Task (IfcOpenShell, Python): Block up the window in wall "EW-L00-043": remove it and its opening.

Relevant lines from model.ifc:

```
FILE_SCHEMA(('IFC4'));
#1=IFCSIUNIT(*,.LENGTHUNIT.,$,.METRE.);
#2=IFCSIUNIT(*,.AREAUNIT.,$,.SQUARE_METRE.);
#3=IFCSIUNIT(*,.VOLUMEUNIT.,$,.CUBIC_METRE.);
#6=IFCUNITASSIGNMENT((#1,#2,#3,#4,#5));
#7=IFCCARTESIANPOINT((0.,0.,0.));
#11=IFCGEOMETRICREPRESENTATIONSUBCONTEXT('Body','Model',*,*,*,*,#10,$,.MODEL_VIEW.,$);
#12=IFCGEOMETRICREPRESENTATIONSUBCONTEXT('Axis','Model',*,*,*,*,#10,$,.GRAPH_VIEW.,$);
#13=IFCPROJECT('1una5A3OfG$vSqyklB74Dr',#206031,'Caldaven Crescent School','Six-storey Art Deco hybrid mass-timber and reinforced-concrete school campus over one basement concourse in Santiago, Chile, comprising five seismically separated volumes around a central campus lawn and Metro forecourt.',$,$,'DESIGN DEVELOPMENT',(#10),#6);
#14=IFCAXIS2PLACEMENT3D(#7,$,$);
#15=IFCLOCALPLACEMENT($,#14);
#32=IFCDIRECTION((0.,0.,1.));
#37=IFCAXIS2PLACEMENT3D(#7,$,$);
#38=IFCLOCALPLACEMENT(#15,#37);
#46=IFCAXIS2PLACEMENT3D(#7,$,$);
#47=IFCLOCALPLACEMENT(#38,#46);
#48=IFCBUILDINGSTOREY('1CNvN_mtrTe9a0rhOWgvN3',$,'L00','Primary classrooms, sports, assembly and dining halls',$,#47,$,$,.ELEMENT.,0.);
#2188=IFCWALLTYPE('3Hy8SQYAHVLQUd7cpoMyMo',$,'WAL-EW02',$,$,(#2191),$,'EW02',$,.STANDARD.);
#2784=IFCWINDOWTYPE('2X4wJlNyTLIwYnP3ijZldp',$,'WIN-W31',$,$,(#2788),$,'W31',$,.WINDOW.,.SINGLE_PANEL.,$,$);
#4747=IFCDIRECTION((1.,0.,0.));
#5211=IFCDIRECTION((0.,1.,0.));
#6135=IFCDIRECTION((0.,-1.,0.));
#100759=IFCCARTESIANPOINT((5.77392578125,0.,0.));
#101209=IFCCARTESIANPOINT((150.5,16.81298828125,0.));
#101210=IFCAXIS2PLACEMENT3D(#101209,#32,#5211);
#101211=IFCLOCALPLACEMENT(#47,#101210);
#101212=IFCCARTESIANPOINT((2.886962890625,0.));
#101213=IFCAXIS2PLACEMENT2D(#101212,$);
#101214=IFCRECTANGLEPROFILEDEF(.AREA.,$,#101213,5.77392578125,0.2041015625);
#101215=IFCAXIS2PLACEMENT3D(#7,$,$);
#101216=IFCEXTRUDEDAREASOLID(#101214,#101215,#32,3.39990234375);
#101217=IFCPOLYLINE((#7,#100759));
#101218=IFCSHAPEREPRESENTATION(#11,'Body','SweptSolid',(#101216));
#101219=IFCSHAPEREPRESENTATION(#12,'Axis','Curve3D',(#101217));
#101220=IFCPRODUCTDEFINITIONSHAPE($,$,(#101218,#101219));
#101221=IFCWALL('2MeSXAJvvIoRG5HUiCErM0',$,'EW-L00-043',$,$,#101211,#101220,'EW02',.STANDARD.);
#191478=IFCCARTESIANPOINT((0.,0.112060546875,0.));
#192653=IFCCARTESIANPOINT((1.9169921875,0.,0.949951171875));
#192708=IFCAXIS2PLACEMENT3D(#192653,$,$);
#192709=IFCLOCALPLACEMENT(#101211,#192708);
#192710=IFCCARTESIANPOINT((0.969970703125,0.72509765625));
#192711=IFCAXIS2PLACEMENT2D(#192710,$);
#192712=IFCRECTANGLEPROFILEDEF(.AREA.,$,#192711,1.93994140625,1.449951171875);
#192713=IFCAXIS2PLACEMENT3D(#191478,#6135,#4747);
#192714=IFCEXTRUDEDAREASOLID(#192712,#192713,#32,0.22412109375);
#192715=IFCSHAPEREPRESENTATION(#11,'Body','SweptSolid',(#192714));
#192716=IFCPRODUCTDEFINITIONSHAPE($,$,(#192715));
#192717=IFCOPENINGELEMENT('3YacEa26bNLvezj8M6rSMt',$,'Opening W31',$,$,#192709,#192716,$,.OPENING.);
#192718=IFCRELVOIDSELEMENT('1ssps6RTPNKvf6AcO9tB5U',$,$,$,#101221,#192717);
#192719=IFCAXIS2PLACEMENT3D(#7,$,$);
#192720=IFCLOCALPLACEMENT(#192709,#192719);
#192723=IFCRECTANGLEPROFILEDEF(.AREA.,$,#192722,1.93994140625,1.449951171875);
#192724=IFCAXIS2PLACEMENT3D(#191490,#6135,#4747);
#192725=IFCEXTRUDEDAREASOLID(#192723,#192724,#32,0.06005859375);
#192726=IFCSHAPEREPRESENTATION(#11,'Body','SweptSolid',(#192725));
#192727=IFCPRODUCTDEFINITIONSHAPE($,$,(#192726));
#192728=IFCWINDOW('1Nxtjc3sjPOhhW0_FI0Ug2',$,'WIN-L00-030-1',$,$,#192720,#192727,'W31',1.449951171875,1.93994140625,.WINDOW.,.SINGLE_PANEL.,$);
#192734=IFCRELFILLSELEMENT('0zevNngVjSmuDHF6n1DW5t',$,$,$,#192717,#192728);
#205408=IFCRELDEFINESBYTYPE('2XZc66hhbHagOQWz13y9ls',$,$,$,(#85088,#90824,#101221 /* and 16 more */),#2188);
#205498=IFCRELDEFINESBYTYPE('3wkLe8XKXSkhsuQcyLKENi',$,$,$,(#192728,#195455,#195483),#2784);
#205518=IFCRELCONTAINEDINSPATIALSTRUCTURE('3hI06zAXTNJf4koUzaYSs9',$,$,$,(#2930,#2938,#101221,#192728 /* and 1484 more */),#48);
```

```python
import ifcopenshell
import ifcopenshell.api.feature
import ifcopenshell.api.root
import ifcopenshell.geom
import ifcopenshell.util.shape

model = ifcopenshell.open("model.ifc")
settings = ifcopenshell.geom.settings()


def volume(element):
    """Net volume in cubic metres, openings subtracted."""
    shape = ifcopenshell.geom.create_shape(settings, element)
    return ifcopenshell.util.shape.get_volume(shape.geometry)


window = model.by_id(192728)
opening = window.FillsVoids[0].RelatingOpeningElement
wall = opening.VoidsElements[0].RelatingBuildingElement
before = volume(wall)

ifcopenshell.api.root.remove_product(model, product=window)
ifcopenshell.api.feature.remove_feature(model, feature=opening)

after = volume(wall)

print(f"wall volume {before:.3f} -> {after:.3f} m3")

model.write("model-out.ifc")
```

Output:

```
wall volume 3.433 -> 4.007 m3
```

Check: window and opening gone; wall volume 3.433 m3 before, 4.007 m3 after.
